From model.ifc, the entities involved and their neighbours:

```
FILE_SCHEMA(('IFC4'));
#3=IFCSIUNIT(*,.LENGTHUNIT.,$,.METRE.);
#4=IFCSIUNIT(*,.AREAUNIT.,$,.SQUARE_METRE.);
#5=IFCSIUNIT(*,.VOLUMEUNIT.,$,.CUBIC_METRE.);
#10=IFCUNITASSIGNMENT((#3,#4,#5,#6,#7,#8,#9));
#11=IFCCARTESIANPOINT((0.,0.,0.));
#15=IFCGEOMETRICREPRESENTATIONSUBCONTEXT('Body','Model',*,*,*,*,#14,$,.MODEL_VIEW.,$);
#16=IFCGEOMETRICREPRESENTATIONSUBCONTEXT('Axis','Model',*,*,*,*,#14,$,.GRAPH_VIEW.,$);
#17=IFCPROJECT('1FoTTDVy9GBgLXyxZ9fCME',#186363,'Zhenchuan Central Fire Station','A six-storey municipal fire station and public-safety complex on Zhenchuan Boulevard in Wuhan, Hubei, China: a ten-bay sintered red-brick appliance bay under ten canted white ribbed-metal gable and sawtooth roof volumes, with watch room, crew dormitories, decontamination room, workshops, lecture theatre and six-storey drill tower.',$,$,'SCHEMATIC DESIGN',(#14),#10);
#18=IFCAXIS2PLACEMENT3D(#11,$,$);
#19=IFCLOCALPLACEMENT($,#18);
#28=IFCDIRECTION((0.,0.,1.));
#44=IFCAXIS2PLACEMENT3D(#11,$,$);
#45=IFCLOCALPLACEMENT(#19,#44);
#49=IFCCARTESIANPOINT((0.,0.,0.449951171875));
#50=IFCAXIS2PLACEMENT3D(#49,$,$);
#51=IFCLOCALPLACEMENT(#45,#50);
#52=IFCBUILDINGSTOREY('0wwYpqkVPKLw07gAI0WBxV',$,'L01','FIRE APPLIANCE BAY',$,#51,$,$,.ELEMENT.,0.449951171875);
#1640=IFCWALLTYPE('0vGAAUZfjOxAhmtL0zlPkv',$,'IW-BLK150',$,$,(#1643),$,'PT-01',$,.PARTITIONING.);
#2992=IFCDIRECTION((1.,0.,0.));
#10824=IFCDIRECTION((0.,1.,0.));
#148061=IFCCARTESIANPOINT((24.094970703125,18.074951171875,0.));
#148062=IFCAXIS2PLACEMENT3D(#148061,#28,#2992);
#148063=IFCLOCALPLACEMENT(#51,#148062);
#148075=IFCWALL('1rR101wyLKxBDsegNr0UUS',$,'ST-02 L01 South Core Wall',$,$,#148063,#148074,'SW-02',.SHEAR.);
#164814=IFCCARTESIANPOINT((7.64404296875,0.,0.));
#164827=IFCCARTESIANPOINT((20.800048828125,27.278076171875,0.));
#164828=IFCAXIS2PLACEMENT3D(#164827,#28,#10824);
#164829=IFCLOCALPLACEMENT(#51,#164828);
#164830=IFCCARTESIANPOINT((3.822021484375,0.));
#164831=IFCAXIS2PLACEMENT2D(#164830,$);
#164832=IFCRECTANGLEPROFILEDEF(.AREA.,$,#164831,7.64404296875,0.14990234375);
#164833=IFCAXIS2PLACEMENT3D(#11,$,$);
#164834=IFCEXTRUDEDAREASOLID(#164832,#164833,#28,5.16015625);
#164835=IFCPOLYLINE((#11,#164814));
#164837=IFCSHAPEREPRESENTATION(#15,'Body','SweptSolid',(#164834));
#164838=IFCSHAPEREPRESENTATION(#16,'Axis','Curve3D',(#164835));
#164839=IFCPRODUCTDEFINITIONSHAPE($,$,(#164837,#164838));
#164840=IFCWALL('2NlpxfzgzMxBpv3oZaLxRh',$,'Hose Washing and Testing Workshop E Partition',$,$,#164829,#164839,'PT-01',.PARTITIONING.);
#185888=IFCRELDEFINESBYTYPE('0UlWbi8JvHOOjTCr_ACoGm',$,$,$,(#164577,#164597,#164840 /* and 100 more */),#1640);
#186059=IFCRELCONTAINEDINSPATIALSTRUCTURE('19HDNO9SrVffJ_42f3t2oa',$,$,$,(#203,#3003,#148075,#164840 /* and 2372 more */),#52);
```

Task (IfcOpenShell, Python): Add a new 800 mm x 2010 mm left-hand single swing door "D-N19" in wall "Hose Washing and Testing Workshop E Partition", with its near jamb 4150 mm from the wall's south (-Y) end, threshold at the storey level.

```python
import numpy as np
import ifcopenshell
import ifcopenshell.api.feature
import ifcopenshell.api.geometry
import ifcopenshell.api.root
import ifcopenshell.api.spatial
import ifcopenshell.geom
import ifcopenshell.util.element
import ifcopenshell.util.placement
import ifcopenshell.util.representation
import ifcopenshell.util.shape
import ifcopenshell.util.unit

model = ifcopenshell.open("model.ifc")
unit_scale = ifcopenshell.util.unit.calculate_unit_scale(model)
settings = ifcopenshell.geom.settings()


def volume(element):
    """Net volume in cubic metres, openings subtracted."""
    shape = ifcopenshell.geom.create_shape(settings, element)
    return ifcopenshell.util.shape.get_volume(shape.geometry)


wall = model.by_guid("2NlpxfzgzMxBpv3oZaLxRh")
storey = ifcopenshell.util.element.get_container(wall, ifc_class="IfcBuildingStorey")
context = ifcopenshell.util.representation.get_context(model, "Model", "Body", "MODEL_VIEW")
before = volume(wall)

width, height, from_end, sill = 0.8, 2.01, 4.15, 0.0  # metres

# The wall runs along its own X axis, and the end named is its -X end.
wall_shape = ifcopenshell.geom.create_shape(settings, wall)
x, y, z = ifcopenshell.util.shape.get_vertices(wall_shape.geometry).T
start = x.min() + from_end
face, thickness = float(y.min()), float(y.max() - y.min())
wall_matrix = ifcopenshell.util.placement.get_local_placement(wall.ObjectPlacement)
level = ifcopenshell.util.placement.get_local_placement(storey.ObjectPlacement)[2, 3]


def in_wall(x, y):
    """Placement at x, y metres in the wall's axes, at sill height."""
    matrix = wall_matrix.copy()
    matrix[:, 3] = wall_matrix @ np.array([x / unit_scale, y / unit_scale, 0.0, 1.0])
    matrix[2, 3] = level + sill / unit_scale
    return matrix


# Opening: a box that overshoots both wall faces by 50 mm.
opening = ifcopenshell.api.root.create_entity(model, ifc_class="IfcOpeningElement", predefined_type="OPENING")
box = ifcopenshell.api.geometry.add_wall_representation(
    model, context=context, length=width, height=height, thickness=thickness + 0.1
)
ifcopenshell.api.geometry.assign_representation(model, product=opening, representation=box)
ifcopenshell.api.geometry.edit_object_placement(model, product=opening, matrix=in_wall(start, face - 0.05), is_si=False)
ifcopenshell.api.feature.add_feature(model, feature=opening, element=wall)

door = ifcopenshell.api.root.create_entity(model, ifc_class="IfcDoor", name="D-N19", predefined_type="DOOR")
door.OverallWidth, door.OverallHeight = width / unit_scale, height / unit_scale
door.OperationType = "SINGLE_SWING_LEFT"
body = ifcopenshell.api.geometry.add_door_representation(
    model,
    context=context,
    overall_width=door.OverallWidth,
    overall_height=door.OverallHeight,
    operation_type="SINGLE_SWING_LEFT",
    lining_properties={"LiningDepth": thickness / unit_scale, "ThresholdDepth": thickness / unit_scale},
)
ifcopenshell.api.geometry.assign_representation(model, product=door, representation=body)
ifcopenshell.api.spatial.assign_container(model, products=[door], relating_structure=storey)
ifcopenshell.api.feature.add_filling(model, opening=opening, element=door)

# The lining spans the wall, so the door starts at the wall face.
ifcopenshell.api.geometry.edit_object_placement(model, product=door, matrix=in_wall(start, face), is_si=False)

after = volume(wall)

print(f"wall volume {before:.3f} -> {after:.3f} m3")

model.write("model_updated.ifc")
```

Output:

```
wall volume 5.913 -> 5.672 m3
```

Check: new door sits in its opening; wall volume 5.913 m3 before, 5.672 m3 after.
